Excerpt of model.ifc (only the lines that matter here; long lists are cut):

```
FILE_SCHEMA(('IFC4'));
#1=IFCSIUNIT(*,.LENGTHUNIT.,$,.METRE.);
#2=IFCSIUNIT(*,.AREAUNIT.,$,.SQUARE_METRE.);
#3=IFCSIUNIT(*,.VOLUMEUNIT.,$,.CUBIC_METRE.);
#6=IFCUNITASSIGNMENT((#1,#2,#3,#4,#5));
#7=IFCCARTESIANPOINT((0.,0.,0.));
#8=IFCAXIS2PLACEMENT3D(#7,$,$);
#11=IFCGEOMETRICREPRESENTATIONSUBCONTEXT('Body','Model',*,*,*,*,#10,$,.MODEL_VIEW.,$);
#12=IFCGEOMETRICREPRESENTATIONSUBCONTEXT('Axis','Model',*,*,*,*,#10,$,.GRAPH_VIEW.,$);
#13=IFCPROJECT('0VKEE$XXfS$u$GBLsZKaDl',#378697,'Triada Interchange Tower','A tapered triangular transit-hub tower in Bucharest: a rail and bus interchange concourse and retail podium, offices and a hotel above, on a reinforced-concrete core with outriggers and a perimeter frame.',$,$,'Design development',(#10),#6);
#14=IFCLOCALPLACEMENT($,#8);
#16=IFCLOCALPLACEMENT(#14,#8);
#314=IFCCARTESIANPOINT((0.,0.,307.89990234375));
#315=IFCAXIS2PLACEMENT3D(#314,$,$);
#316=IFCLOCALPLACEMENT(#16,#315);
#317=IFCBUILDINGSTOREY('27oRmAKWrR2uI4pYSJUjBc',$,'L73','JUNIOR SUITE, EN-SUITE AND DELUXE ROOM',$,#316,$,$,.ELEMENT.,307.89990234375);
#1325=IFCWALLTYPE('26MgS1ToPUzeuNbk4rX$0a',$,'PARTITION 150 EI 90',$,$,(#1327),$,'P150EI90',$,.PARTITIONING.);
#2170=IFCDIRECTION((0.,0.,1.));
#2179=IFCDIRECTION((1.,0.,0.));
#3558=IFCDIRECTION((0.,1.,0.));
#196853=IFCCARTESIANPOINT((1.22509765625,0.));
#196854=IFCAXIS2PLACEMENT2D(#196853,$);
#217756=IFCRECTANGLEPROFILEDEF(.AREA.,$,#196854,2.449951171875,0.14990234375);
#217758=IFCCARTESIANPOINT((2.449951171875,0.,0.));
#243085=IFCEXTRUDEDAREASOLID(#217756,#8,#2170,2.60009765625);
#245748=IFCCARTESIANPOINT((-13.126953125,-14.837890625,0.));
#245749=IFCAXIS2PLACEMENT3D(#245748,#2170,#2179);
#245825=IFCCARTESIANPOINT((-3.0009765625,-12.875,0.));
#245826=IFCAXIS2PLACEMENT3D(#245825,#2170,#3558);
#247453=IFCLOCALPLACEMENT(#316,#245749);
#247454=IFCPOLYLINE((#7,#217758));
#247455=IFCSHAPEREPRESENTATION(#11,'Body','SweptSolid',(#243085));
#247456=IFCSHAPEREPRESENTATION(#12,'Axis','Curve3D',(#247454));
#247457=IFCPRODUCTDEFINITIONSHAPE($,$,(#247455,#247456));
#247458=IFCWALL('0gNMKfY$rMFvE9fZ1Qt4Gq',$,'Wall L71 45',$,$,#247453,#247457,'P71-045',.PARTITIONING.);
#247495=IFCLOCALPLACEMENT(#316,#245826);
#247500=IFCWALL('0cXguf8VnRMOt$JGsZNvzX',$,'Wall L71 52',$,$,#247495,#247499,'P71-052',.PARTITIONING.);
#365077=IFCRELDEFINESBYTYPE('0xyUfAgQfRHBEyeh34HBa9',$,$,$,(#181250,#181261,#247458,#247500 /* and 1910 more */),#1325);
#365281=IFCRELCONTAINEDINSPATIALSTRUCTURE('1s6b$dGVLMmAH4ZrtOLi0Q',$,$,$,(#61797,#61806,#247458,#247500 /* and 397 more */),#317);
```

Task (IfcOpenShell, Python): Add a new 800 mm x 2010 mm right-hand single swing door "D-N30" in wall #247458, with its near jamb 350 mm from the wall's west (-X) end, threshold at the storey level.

```python
import numpy as np
import ifcopenshell
import ifcopenshell.api.feature
import ifcopenshell.api.geometry
import ifcopenshell.api.root
import ifcopenshell.api.spatial
import ifcopenshell.geom
import ifcopenshell.util.element
import ifcopenshell.util.placement
import ifcopenshell.util.representation
import ifcopenshell.util.shape
import ifcopenshell.util.unit

model = ifcopenshell.open("model.ifc")
unit_scale = ifcopenshell.util.unit.calculate_unit_scale(model)
settings = ifcopenshell.geom.settings()


def volume(element):
    """Net volume in cubic metres, openings subtracted."""
    shape = ifcopenshell.geom.create_shape(settings, element)
    return ifcopenshell.util.shape.get_volume(shape.geometry)


wall = model.by_id(247458)
storey = ifcopenshell.util.element.get_container(wall, ifc_class="IfcBuildingStorey")
context = ifcopenshell.util.representation.get_context(model, "Model", "Body", "MODEL_VIEW")
before = volume(wall)

width, height, from_end, sill = 0.8, 2.01, 0.35, 0.0  # metres

# The wall runs along its own X axis, and the end named is its -X end.
wall_shape = ifcopenshell.geom.create_shape(settings, wall)
x, y, z = ifcopenshell.util.shape.get_vertices(wall_shape.geometry).T
start = x.min() + from_end
face, thickness = float(y.min()), float(y.max() - y.min())
wall_matrix = ifcopenshell.util.placement.get_local_placement(wall.ObjectPlacement)
level = ifcopenshell.util.placement.get_local_placement(storey.ObjectPlacement)[2, 3]


def in_wall(x, y):
    """Placement at x, y metres in the wall's axes, at sill height."""
    matrix = wall_matrix.copy()
    matrix[:, 3] = wall_matrix @ np.array([x / unit_scale, y / unit_scale, 0.0, 1.0])
    matrix[2, 3] = level + sill / unit_scale
    return matrix


# Opening: a box that overshoots both wall faces by 50 mm.
opening = ifcopenshell.api.root.create_entity(model, ifc_class="IfcOpeningElement", predefined_type="OPENING")
box = ifcopenshell.api.geometry.add_wall_representation(
    model, context=context, length=width, height=height, thickness=thickness + 0.1
)
ifcopenshell.api.geometry.assign_representation(model, product=opening, representation=box)
ifcopenshell.api.geometry.edit_object_placement(model, product=opening, matrix=in_wall(start, face - 0.05), is_si=False)
ifcopenshell.api.feature.add_feature(model, feature=opening, element=wall)

door = ifcopenshell.api.root.create_entity(model, ifc_class="IfcDoor", name="D-N30", predefined_type="DOOR")
door.OverallWidth, door.OverallHeight = width / unit_scale, height / unit_scale
door.OperationType = "SINGLE_SWING_RIGHT"
body = ifcopenshell.api.geometry.add_door_representation(
    model,
    context=context,
    overall_width=door.OverallWidth,
    overall_height=door.OverallHeight,
    operation_type="SINGLE_SWING_RIGHT",
    lining_properties={"LiningDepth": thickness / unit_scale, "ThresholdDepth": thickness / unit_scale},
)
ifcopenshell.api.geometry.assign_representation(model, product=door, representation=body)
ifcopenshell.api.spatial.assign_container(model, products=[door], relating_structure=storey)
ifcopenshell.api.feature.add_filling(model, opening=opening, element=door)

# The lining spans the wall, so the door starts at the wall face.
ifcopenshell.api.geometry.edit_object_placement(model, product=door, matrix=in_wall(start, face), is_si=False)

after = volume(wall)

print(f"wall volume {before:.3f} -> {after:.3f} m3")

model.write("model_rev.ifc")
```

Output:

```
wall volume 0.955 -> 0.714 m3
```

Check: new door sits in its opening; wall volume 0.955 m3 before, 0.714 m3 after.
